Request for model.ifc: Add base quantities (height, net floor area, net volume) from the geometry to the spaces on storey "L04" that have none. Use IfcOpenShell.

First a look at what the model holds.

```python
import ifcopenshell
import ifcopenshell.util.element
import ifcopenshell.util.unit

model = ifcopenshell.open("model.ifc")
print(model.schema)
for unit_type in ("LENGTHUNIT", "AREAUNIT", "VOLUMEUNIT"):
    print(unit_type, ifcopenshell.util.unit.calculate_unit_scale(model, unit_type))
storey = next(s for s in model.by_type("IfcBuildingStorey") if s.Name == "L04")
spaces = [e for e in ifcopenshell.util.element.get_decomposition(storey) if e.is_a("IfcSpace")]
for e in sorted(spaces, key=lambda e: e.id()):
    print(e.id(), e.is_a(), e.Name, list(ifcopenshell.util.element.get_psets(e, qtos_only=True)), sep=" | ")
```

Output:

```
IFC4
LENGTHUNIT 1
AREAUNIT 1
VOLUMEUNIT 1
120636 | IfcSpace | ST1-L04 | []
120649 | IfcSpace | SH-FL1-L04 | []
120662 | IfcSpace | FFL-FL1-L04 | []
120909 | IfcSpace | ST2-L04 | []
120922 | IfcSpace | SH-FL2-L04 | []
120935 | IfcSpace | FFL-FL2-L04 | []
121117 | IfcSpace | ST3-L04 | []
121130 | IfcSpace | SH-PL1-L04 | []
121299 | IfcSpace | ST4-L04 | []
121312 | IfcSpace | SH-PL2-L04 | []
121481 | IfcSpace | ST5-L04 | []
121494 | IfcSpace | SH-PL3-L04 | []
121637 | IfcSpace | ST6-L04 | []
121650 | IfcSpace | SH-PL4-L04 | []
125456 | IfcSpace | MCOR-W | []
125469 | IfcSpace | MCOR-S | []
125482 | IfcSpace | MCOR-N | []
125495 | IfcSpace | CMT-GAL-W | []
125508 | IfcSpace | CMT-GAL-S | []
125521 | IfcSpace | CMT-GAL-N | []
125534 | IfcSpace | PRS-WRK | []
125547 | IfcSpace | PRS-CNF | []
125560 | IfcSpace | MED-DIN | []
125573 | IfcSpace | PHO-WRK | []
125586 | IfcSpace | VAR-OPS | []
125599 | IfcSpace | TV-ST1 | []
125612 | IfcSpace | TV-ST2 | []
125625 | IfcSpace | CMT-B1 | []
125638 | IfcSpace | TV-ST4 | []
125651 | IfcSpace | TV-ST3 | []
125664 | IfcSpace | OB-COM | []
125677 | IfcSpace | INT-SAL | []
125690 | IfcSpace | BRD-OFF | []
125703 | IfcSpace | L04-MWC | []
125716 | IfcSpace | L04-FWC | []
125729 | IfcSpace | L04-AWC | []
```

```python
import ifcopenshell
import ifcopenshell.api.pset
import ifcopenshell.geom
import ifcopenshell.util.element
import ifcopenshell.util.shape
import ifcopenshell.util.unit

model = ifcopenshell.open("model.ifc")
unit_scale = ifcopenshell.util.unit.calculate_unit_scale(model)
area_scale = ifcopenshell.util.unit.calculate_unit_scale(model, "AREAUNIT")
volume_scale = ifcopenshell.util.unit.calculate_unit_scale(model, "VOLUMEUNIT")
settings = ifcopenshell.geom.settings()

storey = next(s for s in model.by_type("IfcBuildingStorey") if s.Name == "L04")
spaces = [e for e in ifcopenshell.util.element.get_decomposition(storey) if e.is_a("IfcSpace")]

for e in sorted(spaces, key=lambda e: e.id()):
    if ifcopenshell.util.element.get_psets(e, qtos_only=True, should_inherit=False):
        continue
    # Geometry comes back in metres, in the element's own axes.
    shape = ifcopenshell.geom.create_shape(settings, e)
    values = {
        "Height": ifcopenshell.util.shape.get_z(shape.geometry) / unit_scale,
        "NetFloorArea": ifcopenshell.util.shape.get_footprint_area(shape.geometry) / area_scale,
        "NetVolume": ifcopenshell.util.shape.get_volume(shape.geometry) / volume_scale,
    }
    qto = ifcopenshell.api.pset.add_qto(model, product=e, name="Qto_SpaceBaseQuantities")
    ifcopenshell.api.pset.edit_qto(model, qto=qto, properties=values)
    print(e.id(), {k: round(v, 3) for k, v in values.items()})

model.write("model_edited.ifc")
```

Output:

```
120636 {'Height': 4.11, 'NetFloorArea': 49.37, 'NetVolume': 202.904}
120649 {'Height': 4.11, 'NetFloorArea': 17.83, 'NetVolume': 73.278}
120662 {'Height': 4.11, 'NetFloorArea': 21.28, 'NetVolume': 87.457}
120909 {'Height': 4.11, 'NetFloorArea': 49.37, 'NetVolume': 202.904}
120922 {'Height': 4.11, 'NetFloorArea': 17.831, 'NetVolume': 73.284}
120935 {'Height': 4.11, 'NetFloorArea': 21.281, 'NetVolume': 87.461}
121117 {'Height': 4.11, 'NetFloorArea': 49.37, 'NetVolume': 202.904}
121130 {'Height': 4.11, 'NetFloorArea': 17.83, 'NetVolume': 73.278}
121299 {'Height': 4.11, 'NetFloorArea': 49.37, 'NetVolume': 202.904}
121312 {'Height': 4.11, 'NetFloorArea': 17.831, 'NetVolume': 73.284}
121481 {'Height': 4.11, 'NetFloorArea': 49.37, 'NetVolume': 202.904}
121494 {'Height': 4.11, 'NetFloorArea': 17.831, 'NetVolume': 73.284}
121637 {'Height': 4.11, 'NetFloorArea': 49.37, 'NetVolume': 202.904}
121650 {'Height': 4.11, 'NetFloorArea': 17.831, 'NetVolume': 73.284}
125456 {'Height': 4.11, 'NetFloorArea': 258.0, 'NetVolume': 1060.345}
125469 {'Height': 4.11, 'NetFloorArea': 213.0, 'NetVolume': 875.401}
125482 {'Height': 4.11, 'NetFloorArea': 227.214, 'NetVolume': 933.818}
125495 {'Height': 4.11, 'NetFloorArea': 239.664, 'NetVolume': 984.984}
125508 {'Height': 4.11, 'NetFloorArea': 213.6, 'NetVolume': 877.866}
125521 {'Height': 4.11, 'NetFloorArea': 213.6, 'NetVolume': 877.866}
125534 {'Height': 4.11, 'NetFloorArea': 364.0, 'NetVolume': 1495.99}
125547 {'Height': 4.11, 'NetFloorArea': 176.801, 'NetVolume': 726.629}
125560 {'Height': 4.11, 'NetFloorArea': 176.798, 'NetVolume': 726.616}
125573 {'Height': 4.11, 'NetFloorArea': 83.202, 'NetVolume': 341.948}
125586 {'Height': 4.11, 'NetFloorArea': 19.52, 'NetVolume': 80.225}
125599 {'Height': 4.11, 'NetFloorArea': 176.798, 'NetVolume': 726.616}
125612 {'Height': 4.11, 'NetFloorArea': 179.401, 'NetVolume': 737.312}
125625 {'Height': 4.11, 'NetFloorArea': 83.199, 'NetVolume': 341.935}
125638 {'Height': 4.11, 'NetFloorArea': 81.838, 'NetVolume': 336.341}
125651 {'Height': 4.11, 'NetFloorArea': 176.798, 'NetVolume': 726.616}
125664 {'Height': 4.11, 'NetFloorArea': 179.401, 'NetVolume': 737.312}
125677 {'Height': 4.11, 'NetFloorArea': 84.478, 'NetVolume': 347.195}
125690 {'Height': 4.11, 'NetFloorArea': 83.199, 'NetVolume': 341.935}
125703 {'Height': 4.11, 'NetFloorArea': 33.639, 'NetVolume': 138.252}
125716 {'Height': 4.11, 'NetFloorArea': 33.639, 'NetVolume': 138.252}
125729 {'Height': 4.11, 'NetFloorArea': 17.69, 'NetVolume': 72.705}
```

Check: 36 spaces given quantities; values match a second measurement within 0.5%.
